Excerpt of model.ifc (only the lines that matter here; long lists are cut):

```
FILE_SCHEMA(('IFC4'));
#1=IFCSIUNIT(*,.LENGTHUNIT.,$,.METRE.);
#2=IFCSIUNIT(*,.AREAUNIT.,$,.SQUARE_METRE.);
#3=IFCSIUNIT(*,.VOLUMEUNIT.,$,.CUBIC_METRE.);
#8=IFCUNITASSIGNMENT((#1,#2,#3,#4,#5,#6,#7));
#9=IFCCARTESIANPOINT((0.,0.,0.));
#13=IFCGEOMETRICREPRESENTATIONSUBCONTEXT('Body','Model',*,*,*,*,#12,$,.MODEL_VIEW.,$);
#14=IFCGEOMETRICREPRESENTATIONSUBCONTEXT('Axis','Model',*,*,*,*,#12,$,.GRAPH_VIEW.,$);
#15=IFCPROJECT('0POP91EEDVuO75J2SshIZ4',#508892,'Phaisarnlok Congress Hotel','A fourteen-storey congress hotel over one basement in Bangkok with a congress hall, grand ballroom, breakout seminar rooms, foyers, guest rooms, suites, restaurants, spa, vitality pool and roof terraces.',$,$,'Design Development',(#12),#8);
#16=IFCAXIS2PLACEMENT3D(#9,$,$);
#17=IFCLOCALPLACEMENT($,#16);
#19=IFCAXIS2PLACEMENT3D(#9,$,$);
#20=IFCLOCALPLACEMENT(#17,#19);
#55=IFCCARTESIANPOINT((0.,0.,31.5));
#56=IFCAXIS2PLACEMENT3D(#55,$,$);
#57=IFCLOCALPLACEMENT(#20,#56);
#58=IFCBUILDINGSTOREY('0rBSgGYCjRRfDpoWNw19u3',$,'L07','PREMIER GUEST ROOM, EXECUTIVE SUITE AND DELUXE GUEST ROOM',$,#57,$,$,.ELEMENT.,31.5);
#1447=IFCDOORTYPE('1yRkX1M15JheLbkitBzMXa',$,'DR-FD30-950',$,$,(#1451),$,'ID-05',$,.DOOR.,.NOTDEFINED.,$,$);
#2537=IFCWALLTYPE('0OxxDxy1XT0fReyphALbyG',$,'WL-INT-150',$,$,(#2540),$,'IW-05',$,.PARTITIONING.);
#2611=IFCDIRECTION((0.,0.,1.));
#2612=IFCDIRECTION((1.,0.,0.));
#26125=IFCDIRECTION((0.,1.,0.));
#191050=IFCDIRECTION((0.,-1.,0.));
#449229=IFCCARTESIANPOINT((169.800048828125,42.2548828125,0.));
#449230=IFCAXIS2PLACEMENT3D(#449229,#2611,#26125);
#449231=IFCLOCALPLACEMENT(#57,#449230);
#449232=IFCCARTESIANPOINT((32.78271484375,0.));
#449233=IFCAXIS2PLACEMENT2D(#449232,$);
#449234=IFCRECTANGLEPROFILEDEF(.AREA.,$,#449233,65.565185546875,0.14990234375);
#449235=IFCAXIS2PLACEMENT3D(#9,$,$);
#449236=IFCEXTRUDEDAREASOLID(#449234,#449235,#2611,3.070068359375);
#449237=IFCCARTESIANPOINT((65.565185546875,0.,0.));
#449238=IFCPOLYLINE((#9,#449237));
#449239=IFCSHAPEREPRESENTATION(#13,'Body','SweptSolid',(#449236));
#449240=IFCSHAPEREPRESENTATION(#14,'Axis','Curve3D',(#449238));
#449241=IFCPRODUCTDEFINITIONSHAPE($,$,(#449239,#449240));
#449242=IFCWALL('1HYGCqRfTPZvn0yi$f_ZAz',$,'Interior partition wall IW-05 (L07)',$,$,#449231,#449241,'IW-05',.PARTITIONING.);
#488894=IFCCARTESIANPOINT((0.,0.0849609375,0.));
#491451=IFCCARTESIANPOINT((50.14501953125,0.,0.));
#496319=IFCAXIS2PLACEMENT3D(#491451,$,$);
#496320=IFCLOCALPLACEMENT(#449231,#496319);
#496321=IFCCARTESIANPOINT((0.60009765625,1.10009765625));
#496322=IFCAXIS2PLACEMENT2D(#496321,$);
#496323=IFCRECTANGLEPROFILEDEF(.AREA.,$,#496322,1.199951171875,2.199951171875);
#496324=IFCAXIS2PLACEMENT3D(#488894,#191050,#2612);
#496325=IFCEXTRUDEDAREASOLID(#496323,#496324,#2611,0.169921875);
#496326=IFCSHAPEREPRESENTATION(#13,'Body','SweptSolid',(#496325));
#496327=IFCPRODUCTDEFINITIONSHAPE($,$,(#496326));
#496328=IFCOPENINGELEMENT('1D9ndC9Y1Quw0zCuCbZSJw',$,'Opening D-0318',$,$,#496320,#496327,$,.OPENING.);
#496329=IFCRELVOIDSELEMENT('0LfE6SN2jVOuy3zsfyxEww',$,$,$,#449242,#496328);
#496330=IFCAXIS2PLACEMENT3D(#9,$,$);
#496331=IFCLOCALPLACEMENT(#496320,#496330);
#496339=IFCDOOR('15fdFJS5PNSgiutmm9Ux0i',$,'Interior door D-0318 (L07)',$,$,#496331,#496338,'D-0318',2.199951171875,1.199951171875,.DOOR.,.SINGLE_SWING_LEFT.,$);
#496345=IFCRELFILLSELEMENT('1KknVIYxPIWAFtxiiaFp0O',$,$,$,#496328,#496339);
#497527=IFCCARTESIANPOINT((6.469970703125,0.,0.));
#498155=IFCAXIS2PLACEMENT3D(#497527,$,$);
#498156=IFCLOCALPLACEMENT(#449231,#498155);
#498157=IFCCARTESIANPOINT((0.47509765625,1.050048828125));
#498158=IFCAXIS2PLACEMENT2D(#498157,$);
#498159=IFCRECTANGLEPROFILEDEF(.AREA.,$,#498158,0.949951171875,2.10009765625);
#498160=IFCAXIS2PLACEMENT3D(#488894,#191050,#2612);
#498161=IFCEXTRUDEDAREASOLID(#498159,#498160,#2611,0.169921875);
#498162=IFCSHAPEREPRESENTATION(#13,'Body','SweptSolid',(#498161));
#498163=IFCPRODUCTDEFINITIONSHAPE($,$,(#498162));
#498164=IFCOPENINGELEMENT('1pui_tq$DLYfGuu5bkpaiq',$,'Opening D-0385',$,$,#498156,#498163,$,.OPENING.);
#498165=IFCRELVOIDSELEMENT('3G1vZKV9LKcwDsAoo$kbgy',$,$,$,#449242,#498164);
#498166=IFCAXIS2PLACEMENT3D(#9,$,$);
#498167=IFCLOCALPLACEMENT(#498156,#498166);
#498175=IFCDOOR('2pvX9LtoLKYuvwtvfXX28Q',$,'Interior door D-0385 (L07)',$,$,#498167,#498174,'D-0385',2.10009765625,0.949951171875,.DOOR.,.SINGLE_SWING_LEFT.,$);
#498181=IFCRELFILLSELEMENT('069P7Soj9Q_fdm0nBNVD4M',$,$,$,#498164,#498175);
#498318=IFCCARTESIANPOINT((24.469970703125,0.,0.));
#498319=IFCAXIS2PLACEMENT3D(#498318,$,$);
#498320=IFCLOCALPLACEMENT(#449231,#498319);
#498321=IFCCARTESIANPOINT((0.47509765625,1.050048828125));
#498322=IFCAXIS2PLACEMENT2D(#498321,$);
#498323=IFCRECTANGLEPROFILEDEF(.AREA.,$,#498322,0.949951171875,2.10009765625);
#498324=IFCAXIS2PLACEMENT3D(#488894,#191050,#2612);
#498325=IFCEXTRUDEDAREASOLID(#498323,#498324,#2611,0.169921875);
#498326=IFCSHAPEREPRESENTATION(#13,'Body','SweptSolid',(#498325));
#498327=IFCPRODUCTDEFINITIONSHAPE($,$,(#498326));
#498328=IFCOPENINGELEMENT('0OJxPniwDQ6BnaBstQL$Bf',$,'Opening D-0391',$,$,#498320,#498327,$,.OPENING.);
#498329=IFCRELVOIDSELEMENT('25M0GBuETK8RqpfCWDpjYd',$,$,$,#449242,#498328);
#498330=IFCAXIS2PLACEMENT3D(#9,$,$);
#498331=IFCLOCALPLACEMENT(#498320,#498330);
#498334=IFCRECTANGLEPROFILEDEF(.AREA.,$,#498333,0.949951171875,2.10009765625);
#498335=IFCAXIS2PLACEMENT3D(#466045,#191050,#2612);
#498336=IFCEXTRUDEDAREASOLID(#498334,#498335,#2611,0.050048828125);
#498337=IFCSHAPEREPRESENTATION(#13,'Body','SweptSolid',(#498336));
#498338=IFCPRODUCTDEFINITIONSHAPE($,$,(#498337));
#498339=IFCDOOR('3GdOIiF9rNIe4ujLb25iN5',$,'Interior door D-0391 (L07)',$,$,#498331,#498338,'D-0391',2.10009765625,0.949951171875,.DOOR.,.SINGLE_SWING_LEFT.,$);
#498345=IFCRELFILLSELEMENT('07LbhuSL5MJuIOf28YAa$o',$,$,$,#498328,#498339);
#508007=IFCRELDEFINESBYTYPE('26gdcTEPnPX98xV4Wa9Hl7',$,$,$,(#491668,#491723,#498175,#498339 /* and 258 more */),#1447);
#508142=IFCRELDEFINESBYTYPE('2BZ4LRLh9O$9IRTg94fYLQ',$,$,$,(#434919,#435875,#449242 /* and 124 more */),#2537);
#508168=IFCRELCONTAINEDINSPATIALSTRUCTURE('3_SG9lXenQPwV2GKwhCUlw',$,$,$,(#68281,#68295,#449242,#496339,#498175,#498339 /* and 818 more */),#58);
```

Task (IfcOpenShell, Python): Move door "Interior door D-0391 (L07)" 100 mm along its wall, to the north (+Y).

```python
import ifcopenshell
import ifcopenshell.api.geometry
import ifcopenshell.util.placement

model = ifcopenshell.open("model.ifc")

door = model.by_guid("3GdOIiF9rNIe4ujLb25iN5")
opening = door.FillsVoids[0].RelatingOpeningElement
wall = opening.VoidsElements[0].RelatingBuildingElement

wall_matrix = ifcopenshell.util.placement.get_local_placement(wall.ObjectPlacement)
shift = wall_matrix[:3, 0] * 0.1
before = ifcopenshell.util.placement.get_local_placement(door.ObjectPlacement)[:3, 3].copy()

# The door is placed relative to its opening, so it follows when the opening moves.
matrix = ifcopenshell.util.placement.get_local_placement(opening.ObjectPlacement)
matrix[:3, 3] += shift
ifcopenshell.api.geometry.edit_object_placement(
    model, product=opening, matrix=matrix, is_si=False, should_transform_children=True
)

after = ifcopenshell.util.placement.get_local_placement(door.ObjectPlacement)[:3, 3]
print("door moved by", (after - before).round(3) + 0.0)

model.write("model_updated.ifc")
```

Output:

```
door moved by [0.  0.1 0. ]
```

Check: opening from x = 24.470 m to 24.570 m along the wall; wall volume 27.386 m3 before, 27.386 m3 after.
